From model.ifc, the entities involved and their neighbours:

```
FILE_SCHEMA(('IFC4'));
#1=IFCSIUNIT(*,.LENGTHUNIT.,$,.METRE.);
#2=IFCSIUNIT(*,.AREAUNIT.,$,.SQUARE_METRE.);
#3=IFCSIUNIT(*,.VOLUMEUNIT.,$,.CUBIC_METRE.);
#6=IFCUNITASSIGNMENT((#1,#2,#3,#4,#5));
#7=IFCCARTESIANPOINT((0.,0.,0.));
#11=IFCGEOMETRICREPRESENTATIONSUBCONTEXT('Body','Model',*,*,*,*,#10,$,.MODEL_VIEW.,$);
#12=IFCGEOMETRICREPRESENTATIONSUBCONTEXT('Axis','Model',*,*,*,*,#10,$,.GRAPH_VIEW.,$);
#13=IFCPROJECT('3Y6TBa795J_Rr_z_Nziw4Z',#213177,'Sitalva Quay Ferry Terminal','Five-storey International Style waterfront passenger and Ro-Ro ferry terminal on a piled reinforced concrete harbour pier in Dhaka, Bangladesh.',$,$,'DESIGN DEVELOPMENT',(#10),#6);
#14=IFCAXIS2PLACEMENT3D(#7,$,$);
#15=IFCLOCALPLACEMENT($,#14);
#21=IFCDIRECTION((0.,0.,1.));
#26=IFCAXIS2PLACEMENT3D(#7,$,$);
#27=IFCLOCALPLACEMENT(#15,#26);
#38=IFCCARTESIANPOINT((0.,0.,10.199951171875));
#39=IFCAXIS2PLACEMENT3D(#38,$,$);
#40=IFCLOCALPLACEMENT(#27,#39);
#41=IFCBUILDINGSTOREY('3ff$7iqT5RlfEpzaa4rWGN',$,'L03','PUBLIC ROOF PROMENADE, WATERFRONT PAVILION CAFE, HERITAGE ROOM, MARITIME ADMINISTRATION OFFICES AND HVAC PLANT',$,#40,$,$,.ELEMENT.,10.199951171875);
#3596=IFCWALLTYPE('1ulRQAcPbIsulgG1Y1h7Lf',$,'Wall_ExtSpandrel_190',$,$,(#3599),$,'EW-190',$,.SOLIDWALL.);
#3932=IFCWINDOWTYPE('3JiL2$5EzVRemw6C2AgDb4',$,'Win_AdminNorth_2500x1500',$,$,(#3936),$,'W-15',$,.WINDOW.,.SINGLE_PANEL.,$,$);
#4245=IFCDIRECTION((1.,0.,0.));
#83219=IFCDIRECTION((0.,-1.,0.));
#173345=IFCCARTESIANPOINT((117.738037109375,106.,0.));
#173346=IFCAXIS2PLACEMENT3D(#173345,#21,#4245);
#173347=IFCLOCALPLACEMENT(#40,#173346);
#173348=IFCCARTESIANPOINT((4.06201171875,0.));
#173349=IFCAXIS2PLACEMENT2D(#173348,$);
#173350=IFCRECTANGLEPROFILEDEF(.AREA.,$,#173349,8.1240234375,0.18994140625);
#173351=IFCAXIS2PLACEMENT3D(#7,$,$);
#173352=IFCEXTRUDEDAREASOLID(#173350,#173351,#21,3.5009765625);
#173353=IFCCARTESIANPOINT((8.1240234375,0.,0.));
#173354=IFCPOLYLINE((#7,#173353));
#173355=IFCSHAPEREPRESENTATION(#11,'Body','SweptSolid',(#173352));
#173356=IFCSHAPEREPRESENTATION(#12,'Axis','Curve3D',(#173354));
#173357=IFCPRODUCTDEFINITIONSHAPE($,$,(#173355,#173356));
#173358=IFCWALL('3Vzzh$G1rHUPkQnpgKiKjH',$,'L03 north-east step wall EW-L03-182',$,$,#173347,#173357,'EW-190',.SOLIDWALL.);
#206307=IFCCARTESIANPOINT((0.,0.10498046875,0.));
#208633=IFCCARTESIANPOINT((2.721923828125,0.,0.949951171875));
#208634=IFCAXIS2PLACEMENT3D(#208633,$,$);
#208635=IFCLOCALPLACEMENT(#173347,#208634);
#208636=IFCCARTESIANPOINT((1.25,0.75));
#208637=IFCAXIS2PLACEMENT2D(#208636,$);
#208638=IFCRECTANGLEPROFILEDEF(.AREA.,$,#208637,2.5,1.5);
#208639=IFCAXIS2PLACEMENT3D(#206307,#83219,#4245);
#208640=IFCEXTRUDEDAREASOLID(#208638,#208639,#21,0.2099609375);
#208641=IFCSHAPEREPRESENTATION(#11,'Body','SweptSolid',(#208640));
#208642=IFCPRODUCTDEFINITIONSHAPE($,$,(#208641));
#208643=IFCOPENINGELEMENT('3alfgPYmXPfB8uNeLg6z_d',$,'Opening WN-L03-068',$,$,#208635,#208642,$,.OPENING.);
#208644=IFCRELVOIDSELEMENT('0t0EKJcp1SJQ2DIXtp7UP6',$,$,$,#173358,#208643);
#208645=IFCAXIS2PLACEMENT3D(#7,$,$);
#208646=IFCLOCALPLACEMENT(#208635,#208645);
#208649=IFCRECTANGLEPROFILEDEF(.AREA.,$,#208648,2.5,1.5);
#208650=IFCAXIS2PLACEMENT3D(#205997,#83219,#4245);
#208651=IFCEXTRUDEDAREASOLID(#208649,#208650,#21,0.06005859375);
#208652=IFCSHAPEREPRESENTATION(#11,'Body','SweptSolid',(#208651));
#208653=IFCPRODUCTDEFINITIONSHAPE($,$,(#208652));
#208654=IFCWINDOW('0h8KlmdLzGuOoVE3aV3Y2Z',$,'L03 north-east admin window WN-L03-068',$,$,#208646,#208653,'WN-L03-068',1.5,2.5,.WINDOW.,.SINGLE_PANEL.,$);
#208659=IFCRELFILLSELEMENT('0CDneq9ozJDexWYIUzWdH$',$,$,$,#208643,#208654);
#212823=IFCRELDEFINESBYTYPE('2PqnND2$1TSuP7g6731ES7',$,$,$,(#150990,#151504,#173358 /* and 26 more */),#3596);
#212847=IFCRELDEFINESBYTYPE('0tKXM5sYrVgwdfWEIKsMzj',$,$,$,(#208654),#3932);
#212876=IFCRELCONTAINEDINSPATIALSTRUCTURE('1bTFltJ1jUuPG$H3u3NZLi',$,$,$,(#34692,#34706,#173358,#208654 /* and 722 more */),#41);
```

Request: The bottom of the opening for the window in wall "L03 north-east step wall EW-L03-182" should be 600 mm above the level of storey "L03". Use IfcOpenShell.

```python
import numpy as np
import ifcopenshell
import ifcopenshell.api.geometry
import ifcopenshell.geom
import ifcopenshell.util.element
import ifcopenshell.util.placement
import ifcopenshell.util.shape
import ifcopenshell.util.unit

model = ifcopenshell.open("model.ifc")
unit_scale = ifcopenshell.util.unit.calculate_unit_scale(model)

window = model.by_guid("0h8KlmdLzGuOoVE3aV3Y2Z")
opening = window.FillsVoids[0].RelatingOpeningElement
storey = ifcopenshell.util.element.get_container(window, ifc_class="IfcBuildingStorey")
level = ifcopenshell.util.placement.get_local_placement(storey.ObjectPlacement)[2, 3]

# The opening's origin need not be at the sill, so measure its lowest point.
shape = ifcopenshell.geom.create_shape(ifcopenshell.geom.settings(), opening)
bottom = ifcopenshell.util.shape.get_shape_bottom_elevation(shape, shape.geometry) / unit_scale
dz = level + 0.6 / unit_scale - bottom

shift = np.array([0.0, 0.0, dz])
# The window is placed relative to its opening, so it follows when the opening moves.
matrix = ifcopenshell.util.placement.get_local_placement(opening.ObjectPlacement)
matrix[:3, 3] += shift
ifcopenshell.api.geometry.edit_object_placement(
    model, product=opening, matrix=matrix, is_si=False, should_transform_children=True
)

print(f"moved by {dz * unit_scale:+.3f} m")

model.write("model-out.ifc")
```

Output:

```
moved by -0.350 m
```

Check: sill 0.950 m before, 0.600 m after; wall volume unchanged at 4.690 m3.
